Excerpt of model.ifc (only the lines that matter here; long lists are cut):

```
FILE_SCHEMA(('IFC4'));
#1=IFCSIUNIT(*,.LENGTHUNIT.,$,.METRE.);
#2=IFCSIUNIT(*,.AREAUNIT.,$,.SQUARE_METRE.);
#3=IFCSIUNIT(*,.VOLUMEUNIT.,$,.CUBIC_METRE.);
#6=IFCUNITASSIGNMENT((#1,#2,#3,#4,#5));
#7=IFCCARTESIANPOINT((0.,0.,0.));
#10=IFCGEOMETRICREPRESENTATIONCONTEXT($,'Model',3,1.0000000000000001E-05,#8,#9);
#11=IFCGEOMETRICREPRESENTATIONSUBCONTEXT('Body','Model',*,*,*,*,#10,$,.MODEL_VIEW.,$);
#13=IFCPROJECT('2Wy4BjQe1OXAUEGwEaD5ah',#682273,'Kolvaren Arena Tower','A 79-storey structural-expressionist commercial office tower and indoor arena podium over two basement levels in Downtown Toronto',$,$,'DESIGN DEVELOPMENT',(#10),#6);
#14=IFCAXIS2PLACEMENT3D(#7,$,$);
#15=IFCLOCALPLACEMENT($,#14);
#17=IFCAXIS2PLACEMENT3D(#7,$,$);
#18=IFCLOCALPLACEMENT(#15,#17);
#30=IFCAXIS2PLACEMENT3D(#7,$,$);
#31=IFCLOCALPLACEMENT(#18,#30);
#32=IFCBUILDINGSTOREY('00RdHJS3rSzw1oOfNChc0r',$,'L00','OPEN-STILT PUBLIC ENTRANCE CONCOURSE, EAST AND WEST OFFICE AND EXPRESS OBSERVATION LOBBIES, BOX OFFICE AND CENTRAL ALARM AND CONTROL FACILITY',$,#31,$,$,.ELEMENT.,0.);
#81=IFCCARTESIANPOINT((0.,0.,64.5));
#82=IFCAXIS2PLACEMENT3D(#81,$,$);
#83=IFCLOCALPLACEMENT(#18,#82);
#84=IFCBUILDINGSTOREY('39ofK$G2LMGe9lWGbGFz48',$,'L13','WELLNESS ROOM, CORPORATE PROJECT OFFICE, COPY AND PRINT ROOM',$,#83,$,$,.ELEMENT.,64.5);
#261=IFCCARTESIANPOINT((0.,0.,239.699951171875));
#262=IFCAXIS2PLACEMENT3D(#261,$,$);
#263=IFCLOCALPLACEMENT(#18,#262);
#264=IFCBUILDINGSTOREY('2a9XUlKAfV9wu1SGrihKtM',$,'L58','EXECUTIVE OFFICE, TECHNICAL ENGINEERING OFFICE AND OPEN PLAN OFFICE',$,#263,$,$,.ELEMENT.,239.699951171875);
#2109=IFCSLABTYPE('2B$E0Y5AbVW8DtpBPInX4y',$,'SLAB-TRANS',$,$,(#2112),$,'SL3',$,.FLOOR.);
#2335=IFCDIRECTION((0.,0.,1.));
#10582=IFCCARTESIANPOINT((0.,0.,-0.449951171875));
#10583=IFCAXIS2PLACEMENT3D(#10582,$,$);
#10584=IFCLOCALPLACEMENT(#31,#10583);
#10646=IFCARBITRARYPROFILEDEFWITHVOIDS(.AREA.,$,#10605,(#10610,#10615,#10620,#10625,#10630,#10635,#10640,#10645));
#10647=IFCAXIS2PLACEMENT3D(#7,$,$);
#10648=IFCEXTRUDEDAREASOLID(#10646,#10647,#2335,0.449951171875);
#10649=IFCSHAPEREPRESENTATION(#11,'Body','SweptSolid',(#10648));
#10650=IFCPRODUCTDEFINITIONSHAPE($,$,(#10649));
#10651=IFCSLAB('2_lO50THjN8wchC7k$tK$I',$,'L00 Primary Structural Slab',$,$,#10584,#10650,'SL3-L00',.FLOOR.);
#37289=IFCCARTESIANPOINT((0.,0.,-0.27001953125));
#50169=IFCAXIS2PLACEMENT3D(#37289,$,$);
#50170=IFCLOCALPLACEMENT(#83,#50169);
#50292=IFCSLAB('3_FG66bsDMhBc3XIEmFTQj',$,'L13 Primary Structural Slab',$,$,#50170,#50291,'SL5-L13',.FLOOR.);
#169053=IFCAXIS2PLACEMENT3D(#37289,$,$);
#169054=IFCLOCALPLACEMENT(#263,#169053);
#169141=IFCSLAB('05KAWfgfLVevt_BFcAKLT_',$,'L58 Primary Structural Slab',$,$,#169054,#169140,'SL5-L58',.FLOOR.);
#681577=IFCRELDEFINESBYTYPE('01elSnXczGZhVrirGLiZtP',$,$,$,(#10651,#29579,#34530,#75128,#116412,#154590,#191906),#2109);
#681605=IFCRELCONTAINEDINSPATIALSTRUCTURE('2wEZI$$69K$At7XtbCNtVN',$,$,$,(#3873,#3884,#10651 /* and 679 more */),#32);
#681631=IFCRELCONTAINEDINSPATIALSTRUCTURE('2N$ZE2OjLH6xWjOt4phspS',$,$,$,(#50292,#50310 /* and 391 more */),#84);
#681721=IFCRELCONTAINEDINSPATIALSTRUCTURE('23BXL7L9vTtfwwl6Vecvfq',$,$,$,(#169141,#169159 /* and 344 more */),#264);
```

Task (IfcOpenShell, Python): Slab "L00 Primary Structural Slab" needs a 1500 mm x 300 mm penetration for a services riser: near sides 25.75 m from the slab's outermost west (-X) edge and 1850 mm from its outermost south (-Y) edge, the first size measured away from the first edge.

```python
import numpy as np
import ifcopenshell
import ifcopenshell.api.feature
import ifcopenshell.api.geometry
import ifcopenshell.api.root
import ifcopenshell.geom
import ifcopenshell.util.placement
import ifcopenshell.util.representation
import ifcopenshell.util.shape
import ifcopenshell.util.unit

model = ifcopenshell.open("model.ifc")
unit_scale = ifcopenshell.util.unit.calculate_unit_scale(model)
settings = ifcopenshell.geom.settings()


def volume(element):
    """Net volume in cubic metres, openings subtracted."""
    shape = ifcopenshell.geom.create_shape(settings, element)
    return ifcopenshell.util.shape.get_volume(shape.geometry)


slab = model.by_guid("2_lO50THjN8wchC7k$tK$I")
before = volume(slab)

# Extent in the slab's own axes, in metres. The edges named are its -X and -Y sides.
slab_shape = ifcopenshell.geom.create_shape(settings, slab)
vertices = ifcopenshell.util.shape.get_vertices(slab_shape.geometry)
x_min, y_min, bottom = vertices.min(axis=0)
top = vertices[:, 2].max()

opening = ifcopenshell.api.root.create_entity(model, ifc_class="IfcOpeningElement", name="Services riser opening", predefined_type="OPENING")
context = ifcopenshell.util.representation.get_context(model, "Model", "Body", "MODEL_VIEW")
width, depth = 1.5, 0.3
outline = [(0.0, 0.0), (width, 0.0), (width, depth), (0.0, depth), (0.0, 0.0)]
# Overshoot both faces by 50 mm so the cut is clean.
shape = ifcopenshell.api.geometry.add_slab_representation(
    model, context=context, depth=top - bottom + 0.1, polyline=outline
)
ifcopenshell.api.geometry.assign_representation(model, product=opening, representation=shape)

matrix = ifcopenshell.util.placement.get_local_placement(slab.ObjectPlacement)
matrix[:, 3] = matrix @ np.append(np.array([x_min + 25.75, y_min + 1.85, bottom - 0.05]) / unit_scale, 1.0)
ifcopenshell.api.geometry.edit_object_placement(model, product=opening, matrix=matrix, is_si=False)
ifcopenshell.api.feature.add_feature(model, feature=opening, element=slab)

after = volume(slab)

print(f"slab volume {before:.3f} -> {after:.3f} m3")

model.write("model_rev.ifc")
```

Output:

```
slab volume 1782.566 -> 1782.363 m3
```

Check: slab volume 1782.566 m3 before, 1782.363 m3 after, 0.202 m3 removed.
